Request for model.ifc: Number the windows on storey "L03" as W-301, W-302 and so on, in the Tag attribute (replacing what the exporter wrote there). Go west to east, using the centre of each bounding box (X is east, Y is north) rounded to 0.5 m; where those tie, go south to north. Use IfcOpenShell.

First a look at what the model holds.

```python
import ifcopenshell
import ifcopenshell.util.element
import ifcopenshell.util.placement

model = ifcopenshell.open("model.ifc")
print(model.schema)
storey = next(s for s in model.by_type("IfcBuildingStorey") if s.Name == "L03")
windows = [e for e in ifcopenshell.util.element.get_decomposition(storey) if e.is_a("IfcWindow")]
for e in sorted(windows, key=lambda e: e.id()):
    origin = ifcopenshell.util.placement.get_local_placement(e.ObjectPlacement)[:3, 3]
    print(e.id(), e.Tag, e.Name, origin.round(2) + 0.0, sep=" | ")
```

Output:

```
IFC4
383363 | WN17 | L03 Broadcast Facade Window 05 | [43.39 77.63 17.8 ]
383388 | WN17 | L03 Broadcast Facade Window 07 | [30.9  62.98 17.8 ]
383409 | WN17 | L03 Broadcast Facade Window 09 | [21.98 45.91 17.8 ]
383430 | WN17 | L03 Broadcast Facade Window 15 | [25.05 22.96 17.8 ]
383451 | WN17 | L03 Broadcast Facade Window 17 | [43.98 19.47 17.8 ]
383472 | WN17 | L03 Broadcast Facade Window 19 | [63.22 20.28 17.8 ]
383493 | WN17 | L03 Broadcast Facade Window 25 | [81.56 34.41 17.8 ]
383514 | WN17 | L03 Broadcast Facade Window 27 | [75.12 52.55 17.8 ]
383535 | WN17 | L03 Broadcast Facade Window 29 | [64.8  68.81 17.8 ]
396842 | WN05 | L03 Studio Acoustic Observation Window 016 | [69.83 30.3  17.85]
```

```python
import ifcopenshell
import ifcopenshell.geom
import ifcopenshell.util.element
import ifcopenshell.util.shape

model = ifcopenshell.open("model.ifc")
settings = ifcopenshell.geom.settings()
settings.set("use-world-coords", True)


def centre(element):
    shape = ifcopenshell.geom.create_shape(settings, element)
    return ifcopenshell.util.shape.get_bbox_centroid(shape.geometry)


storey = next(s for s in model.by_type("IfcBuildingStorey") if s.Name == "L03")
windows = [e for e in ifcopenshell.util.element.get_decomposition(storey) if e.is_a("IfcWindow")]

# Insertion points can sit at a corner or the storey origin, so sort by the geometry (in metres).
centres = {e: centre(e) for e in windows}
windows.sort(key=lambda e: (round(centres[e][0] / 0.5), centres[e][1]))

for i, e in enumerate(windows, start=1):
    number = f"W-3{i:02d}"
    e.Tag = number
    print(e.id(), number)

model.write("model_rev.ifc")
```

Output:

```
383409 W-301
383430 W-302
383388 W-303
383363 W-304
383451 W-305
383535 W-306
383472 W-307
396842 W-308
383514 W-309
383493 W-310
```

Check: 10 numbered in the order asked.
